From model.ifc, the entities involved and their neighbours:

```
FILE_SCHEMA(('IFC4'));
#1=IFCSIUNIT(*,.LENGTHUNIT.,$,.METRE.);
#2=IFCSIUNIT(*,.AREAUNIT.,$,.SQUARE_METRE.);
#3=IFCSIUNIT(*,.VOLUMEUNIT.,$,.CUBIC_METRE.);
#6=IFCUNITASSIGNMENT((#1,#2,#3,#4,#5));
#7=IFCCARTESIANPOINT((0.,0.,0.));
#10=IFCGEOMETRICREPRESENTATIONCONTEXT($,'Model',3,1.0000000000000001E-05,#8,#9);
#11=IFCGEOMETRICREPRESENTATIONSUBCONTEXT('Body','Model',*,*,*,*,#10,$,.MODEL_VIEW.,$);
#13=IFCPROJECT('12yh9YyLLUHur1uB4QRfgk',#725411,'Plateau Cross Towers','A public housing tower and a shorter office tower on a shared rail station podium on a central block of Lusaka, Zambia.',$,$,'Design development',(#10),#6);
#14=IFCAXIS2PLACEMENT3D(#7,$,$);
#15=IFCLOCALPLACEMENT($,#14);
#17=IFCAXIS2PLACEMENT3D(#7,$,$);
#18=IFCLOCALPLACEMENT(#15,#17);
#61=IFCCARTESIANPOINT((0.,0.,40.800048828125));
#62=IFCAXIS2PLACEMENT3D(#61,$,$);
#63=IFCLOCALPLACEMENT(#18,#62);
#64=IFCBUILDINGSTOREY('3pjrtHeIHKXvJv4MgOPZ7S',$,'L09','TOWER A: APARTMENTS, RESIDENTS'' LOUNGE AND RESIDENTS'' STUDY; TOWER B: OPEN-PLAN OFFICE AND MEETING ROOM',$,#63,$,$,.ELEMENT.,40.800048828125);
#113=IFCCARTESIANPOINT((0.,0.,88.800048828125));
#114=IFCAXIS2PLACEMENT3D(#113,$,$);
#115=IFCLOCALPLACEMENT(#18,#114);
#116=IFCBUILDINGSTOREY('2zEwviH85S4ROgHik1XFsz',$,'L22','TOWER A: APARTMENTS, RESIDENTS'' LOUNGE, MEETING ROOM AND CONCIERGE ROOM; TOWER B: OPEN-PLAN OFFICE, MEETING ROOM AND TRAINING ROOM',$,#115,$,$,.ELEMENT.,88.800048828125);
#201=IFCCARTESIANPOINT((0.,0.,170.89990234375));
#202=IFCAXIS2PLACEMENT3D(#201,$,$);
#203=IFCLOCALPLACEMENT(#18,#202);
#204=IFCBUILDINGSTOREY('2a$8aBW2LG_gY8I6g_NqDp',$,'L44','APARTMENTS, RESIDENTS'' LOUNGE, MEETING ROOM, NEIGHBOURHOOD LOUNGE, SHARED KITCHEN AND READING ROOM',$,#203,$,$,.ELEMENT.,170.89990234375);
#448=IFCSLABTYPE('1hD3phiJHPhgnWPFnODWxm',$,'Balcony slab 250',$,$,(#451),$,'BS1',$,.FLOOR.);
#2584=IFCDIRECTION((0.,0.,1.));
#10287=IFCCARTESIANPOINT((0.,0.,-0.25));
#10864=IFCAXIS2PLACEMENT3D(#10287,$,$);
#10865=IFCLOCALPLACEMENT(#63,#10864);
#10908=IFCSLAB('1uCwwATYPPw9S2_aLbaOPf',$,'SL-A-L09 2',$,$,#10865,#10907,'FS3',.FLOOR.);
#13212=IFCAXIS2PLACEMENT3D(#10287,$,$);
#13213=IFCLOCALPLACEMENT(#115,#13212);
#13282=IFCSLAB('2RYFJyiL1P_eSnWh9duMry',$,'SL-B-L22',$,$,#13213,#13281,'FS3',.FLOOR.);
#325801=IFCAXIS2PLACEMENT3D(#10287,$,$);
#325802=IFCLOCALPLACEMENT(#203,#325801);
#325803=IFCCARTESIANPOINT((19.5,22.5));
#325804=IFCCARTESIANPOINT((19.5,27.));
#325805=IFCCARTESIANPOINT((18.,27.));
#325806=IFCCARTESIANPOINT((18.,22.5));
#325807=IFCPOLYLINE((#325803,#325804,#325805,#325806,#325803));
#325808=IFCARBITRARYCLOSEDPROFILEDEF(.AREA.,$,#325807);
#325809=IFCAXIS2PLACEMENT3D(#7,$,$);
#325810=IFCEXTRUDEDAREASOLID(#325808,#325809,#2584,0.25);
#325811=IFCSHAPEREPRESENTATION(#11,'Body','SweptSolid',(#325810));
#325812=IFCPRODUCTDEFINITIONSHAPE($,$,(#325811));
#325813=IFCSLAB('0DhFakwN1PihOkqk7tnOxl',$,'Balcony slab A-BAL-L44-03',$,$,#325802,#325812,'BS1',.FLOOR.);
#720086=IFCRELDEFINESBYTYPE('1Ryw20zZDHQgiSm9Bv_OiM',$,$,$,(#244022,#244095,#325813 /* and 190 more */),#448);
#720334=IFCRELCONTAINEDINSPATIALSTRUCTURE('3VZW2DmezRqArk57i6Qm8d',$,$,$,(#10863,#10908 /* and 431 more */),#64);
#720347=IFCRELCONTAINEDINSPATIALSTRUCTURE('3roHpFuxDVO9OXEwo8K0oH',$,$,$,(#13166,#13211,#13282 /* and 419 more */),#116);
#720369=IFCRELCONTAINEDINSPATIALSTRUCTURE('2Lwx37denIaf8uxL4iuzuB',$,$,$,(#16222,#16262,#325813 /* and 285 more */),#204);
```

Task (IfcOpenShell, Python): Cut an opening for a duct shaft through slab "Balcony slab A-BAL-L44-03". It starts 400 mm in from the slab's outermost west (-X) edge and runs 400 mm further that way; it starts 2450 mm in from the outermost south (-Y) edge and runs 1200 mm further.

```python
import numpy as np
import ifcopenshell
import ifcopenshell.api.feature
import ifcopenshell.api.geometry
import ifcopenshell.api.root
import ifcopenshell.geom
import ifcopenshell.util.placement
import ifcopenshell.util.representation
import ifcopenshell.util.shape
import ifcopenshell.util.unit

model = ifcopenshell.open("model.ifc")
unit_scale = ifcopenshell.util.unit.calculate_unit_scale(model)
settings = ifcopenshell.geom.settings()


def volume(element):
    """Net volume in cubic metres, openings subtracted."""
    shape = ifcopenshell.geom.create_shape(settings, element)
    return ifcopenshell.util.shape.get_volume(shape.geometry)


slab = model.by_guid("0DhFakwN1PihOkqk7tnOxl")
before = volume(slab)

# Extent in the slab's own axes, in metres. The edges named are its -X and -Y sides.
slab_shape = ifcopenshell.geom.create_shape(settings, slab)
vertices = ifcopenshell.util.shape.get_vertices(slab_shape.geometry)
x_min, y_min, bottom = vertices.min(axis=0)
top = vertices[:, 2].max()

opening = ifcopenshell.api.root.create_entity(model, ifc_class="IfcOpeningElement", name="Duct shaft opening", predefined_type="OPENING")
context = ifcopenshell.util.representation.get_context(model, "Model", "Body", "MODEL_VIEW")
width, depth = 0.4, 1.2
outline = [(0.0, 0.0), (width, 0.0), (width, depth), (0.0, depth), (0.0, 0.0)]
# Overshoot both faces by 50 mm so the cut is clean.
shape = ifcopenshell.api.geometry.add_slab_representation(
    model, context=context, depth=top - bottom + 0.1, polyline=outline
)
ifcopenshell.api.geometry.assign_representation(model, product=opening, representation=shape)

matrix = ifcopenshell.util.placement.get_local_placement(slab.ObjectPlacement)
matrix[:, 3] = matrix @ np.append(np.array([x_min + 0.4, y_min + 2.45, bottom - 0.05]) / unit_scale, 1.0)
ifcopenshell.api.geometry.edit_object_placement(model, product=opening, matrix=matrix, is_si=False)
ifcopenshell.api.feature.add_feature(model, feature=opening, element=slab)

after = volume(slab)

print(f"slab volume {before:.3f} -> {after:.3f} m3")

model.write("model-out.ifc")
```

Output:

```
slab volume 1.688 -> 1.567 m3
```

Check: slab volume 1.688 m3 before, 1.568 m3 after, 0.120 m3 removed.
